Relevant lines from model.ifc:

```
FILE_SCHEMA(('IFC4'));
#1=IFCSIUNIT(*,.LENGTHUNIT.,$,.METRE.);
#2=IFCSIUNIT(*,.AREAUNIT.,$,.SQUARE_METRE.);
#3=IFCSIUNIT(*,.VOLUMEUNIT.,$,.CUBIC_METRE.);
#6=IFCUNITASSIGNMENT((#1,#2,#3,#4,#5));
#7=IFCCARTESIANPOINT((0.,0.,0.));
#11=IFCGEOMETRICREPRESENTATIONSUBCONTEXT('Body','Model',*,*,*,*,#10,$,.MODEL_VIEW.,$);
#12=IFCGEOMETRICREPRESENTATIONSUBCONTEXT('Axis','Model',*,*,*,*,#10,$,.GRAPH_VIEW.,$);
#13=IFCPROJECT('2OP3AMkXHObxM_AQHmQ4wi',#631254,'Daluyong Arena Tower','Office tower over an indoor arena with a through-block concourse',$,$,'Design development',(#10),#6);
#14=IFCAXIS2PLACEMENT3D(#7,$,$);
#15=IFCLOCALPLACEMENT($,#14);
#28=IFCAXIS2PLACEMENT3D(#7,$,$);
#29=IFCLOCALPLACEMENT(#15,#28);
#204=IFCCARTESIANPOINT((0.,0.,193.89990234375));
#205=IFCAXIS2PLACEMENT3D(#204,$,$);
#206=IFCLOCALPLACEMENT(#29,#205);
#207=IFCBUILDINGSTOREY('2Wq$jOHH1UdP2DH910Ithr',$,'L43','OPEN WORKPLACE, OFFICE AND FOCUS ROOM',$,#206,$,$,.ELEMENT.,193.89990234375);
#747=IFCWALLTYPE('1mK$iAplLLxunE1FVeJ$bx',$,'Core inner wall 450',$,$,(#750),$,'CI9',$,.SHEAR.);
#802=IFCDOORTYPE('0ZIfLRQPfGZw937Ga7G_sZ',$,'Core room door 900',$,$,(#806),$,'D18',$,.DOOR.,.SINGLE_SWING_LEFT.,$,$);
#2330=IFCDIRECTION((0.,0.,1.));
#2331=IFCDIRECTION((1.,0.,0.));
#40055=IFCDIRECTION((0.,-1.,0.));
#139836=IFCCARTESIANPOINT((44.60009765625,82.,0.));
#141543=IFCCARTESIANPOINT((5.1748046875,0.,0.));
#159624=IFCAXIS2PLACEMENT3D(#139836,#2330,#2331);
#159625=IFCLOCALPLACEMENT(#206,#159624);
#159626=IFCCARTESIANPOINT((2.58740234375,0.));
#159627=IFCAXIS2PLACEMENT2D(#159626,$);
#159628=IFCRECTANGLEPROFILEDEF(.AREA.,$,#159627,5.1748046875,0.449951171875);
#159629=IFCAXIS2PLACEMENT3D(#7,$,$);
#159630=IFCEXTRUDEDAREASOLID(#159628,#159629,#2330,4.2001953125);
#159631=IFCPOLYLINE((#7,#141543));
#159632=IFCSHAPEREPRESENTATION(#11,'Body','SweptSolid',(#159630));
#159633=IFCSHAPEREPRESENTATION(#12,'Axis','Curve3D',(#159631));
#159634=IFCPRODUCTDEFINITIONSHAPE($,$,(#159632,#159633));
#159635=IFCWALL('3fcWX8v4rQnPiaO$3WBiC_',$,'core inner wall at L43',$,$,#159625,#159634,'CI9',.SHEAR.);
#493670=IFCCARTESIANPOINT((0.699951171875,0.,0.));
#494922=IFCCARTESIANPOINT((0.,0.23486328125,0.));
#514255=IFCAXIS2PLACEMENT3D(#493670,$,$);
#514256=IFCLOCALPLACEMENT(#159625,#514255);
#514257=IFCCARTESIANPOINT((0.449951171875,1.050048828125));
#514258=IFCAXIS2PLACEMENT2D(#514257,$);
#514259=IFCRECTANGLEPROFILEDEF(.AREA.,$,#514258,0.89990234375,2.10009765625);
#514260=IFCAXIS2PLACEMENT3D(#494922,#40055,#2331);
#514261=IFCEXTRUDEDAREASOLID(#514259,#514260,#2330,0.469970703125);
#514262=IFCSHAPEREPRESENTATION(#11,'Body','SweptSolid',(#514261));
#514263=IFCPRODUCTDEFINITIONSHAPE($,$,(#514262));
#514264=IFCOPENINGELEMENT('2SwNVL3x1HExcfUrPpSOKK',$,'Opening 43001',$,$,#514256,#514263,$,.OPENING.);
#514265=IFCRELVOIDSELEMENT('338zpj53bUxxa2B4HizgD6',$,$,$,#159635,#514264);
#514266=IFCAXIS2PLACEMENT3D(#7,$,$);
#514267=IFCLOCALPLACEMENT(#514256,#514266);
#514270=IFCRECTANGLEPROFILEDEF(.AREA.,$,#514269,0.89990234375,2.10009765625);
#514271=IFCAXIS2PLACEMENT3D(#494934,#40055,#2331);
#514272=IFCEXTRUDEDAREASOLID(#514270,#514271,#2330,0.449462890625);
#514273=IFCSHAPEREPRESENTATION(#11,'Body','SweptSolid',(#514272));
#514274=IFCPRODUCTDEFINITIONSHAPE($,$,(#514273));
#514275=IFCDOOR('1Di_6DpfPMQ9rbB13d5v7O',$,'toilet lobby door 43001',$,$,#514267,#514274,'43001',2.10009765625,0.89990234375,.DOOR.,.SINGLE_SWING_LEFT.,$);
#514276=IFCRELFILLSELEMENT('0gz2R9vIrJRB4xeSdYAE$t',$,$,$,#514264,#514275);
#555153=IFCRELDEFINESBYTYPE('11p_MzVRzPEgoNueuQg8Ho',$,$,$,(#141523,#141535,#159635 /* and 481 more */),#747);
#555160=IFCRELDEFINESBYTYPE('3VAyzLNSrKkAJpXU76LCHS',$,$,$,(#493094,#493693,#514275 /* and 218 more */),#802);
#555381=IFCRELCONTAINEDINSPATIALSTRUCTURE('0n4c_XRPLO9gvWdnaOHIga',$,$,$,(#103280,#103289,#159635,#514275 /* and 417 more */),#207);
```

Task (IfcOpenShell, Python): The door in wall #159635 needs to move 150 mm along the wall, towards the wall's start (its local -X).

```python
import ifcopenshell
import ifcopenshell.api.geometry
import ifcopenshell.util.placement
import ifcopenshell.util.unit

model = ifcopenshell.open("model.ifc")
unit_scale = ifcopenshell.util.unit.calculate_unit_scale(model)

door = model.by_guid("1Di_6DpfPMQ9rbB13d5v7O")
opening = door.FillsVoids[0].RelatingOpeningElement
wall = opening.VoidsElements[0].RelatingBuildingElement

wall_matrix = ifcopenshell.util.placement.get_local_placement(wall.ObjectPlacement)
shift = wall_matrix[:3, 0] * -0.15 / unit_scale
before = ifcopenshell.util.placement.get_local_placement(door.ObjectPlacement)[:3, 3].copy()

# The door is placed relative to its opening, so it follows when the opening moves.
matrix = ifcopenshell.util.placement.get_local_placement(opening.ObjectPlacement)
matrix[:3, 3] += shift
ifcopenshell.api.geometry.edit_object_placement(
    model, product=opening, matrix=matrix, is_si=False, should_transform_children=True
)

after = ifcopenshell.util.placement.get_local_placement(door.ObjectPlacement)[:3, 3]
print("door moved by", (after - before).round(3) + 0.0)

model.write("model_v2.ifc")
```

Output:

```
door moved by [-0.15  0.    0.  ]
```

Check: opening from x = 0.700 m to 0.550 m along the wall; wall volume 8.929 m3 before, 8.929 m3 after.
